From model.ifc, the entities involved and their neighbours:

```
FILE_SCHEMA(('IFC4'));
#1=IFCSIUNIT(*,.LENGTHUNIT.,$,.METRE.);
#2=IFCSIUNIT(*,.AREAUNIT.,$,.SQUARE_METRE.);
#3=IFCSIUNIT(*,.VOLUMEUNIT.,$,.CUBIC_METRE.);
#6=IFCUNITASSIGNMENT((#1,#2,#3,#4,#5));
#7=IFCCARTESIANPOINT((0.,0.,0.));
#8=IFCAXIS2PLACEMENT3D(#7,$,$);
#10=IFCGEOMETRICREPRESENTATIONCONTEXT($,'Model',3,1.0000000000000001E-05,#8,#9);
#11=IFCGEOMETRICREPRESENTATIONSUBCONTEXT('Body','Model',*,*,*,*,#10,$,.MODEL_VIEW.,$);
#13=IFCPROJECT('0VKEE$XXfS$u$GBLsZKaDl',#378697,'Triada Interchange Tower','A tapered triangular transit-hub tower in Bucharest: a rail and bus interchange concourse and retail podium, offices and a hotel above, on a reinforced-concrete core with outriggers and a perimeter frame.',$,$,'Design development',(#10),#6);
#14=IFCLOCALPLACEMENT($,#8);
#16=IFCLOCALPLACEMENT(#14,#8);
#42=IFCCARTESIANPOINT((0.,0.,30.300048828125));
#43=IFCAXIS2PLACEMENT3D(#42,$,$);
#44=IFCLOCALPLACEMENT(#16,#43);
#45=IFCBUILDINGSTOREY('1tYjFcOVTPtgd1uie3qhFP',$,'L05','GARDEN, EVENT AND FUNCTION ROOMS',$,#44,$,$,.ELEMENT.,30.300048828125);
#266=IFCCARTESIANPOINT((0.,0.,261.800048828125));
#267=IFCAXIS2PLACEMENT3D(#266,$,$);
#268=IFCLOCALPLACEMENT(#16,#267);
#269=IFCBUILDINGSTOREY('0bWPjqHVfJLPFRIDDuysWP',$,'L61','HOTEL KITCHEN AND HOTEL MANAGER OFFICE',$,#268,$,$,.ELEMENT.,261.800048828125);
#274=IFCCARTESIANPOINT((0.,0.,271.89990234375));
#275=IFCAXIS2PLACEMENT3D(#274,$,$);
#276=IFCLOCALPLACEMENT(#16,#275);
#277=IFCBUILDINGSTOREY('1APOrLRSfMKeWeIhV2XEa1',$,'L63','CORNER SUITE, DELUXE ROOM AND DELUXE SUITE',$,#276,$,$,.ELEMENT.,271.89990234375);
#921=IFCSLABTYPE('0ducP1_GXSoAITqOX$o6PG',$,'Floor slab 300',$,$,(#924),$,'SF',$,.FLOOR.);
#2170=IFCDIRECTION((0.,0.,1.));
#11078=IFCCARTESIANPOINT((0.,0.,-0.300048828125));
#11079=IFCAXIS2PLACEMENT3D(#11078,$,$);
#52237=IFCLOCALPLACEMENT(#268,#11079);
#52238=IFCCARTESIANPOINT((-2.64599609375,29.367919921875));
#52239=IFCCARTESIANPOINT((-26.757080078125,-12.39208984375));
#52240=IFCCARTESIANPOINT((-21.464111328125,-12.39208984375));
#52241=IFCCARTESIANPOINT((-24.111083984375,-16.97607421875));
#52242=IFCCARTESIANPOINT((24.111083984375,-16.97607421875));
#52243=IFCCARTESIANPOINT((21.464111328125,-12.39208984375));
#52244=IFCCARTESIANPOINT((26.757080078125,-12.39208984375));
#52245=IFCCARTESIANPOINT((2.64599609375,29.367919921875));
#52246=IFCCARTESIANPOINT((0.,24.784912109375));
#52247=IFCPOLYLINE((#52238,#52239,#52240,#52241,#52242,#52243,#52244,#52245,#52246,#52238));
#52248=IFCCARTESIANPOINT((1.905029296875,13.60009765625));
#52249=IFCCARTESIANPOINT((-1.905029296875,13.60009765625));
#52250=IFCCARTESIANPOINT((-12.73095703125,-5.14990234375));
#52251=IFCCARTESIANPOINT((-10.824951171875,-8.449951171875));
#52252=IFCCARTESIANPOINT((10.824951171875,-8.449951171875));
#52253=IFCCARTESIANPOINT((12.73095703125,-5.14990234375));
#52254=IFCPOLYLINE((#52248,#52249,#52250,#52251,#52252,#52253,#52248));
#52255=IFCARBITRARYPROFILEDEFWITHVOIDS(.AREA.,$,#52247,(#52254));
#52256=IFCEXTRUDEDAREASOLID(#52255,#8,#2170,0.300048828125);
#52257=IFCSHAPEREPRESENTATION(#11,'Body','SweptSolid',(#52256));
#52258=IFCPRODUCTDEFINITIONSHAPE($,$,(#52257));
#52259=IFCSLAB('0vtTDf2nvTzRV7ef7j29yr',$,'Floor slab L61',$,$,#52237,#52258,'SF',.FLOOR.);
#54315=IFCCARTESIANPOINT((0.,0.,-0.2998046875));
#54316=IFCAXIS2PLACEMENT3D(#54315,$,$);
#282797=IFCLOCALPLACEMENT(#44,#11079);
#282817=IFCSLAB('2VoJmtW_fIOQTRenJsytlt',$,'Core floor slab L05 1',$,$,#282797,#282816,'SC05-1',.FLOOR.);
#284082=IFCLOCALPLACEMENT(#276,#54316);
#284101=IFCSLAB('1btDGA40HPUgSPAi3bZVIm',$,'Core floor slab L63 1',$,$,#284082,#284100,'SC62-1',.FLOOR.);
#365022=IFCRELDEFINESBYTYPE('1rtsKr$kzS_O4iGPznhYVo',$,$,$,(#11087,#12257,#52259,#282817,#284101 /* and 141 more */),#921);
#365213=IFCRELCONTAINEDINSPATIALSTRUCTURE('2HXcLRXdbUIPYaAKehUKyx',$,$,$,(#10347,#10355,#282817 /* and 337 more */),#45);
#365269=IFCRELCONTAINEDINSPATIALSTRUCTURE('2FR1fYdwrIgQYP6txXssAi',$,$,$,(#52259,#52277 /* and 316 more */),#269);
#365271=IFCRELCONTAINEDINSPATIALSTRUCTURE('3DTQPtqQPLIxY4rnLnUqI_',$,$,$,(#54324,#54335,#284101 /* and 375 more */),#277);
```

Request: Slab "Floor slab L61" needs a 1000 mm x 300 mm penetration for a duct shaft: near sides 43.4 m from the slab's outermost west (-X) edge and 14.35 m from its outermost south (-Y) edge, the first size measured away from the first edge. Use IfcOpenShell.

```python
import numpy as np
import ifcopenshell
import ifcopenshell.api.feature
import ifcopenshell.api.geometry
import ifcopenshell.api.root
import ifcopenshell.geom
import ifcopenshell.util.placement
import ifcopenshell.util.representation
import ifcopenshell.util.shape
import ifcopenshell.util.unit

model = ifcopenshell.open("model.ifc")
unit_scale = ifcopenshell.util.unit.calculate_unit_scale(model)
settings = ifcopenshell.geom.settings()


def volume(element):
    """Net volume in cubic metres, openings subtracted."""
    shape = ifcopenshell.geom.create_shape(settings, element)
    return ifcopenshell.util.shape.get_volume(shape.geometry)


slab = model.by_guid("0vtTDf2nvTzRV7ef7j29yr")
before = volume(slab)

# Extent in the slab's own axes, in metres. The edges named are its -X and -Y sides.
slab_shape = ifcopenshell.geom.create_shape(settings, slab)
vertices = ifcopenshell.util.shape.get_vertices(slab_shape.geometry)
x_min, y_min, bottom = vertices.min(axis=0)
top = vertices[:, 2].max()

opening = ifcopenshell.api.root.create_entity(model, ifc_class="IfcOpeningElement", name="Duct shaft opening", predefined_type="OPENING")
context = ifcopenshell.util.representation.get_context(model, "Model", "Body", "MODEL_VIEW")
width, depth = 1, 0.3
outline = [(0.0, 0.0), (width, 0.0), (width, depth), (0.0, depth), (0.0, 0.0)]
# Overshoot both faces by 50 mm so the cut is clean.
shape = ifcopenshell.api.geometry.add_slab_representation(
    model, context=context, depth=top - bottom + 0.1, polyline=outline
)
ifcopenshell.api.geometry.assign_representation(model, product=opening, representation=shape)

matrix = ifcopenshell.util.placement.get_local_placement(slab.ObjectPlacement)
matrix[:, 3] = matrix @ np.append(np.array([x_min + 43.4, y_min + 14.35, bottom - 0.05]) / unit_scale, 1.0)
ifcopenshell.api.geometry.edit_object_placement(model, product=opening, matrix=matrix, is_si=False)
ifcopenshell.api.feature.add_feature(model, feature=opening, element=slab)

after = volume(slab)

print(f"slab volume {before:.3f} -> {after:.3f} m3")

model.write("model_v2.ifc")
```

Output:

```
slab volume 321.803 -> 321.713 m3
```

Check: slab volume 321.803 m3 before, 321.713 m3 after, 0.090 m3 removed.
